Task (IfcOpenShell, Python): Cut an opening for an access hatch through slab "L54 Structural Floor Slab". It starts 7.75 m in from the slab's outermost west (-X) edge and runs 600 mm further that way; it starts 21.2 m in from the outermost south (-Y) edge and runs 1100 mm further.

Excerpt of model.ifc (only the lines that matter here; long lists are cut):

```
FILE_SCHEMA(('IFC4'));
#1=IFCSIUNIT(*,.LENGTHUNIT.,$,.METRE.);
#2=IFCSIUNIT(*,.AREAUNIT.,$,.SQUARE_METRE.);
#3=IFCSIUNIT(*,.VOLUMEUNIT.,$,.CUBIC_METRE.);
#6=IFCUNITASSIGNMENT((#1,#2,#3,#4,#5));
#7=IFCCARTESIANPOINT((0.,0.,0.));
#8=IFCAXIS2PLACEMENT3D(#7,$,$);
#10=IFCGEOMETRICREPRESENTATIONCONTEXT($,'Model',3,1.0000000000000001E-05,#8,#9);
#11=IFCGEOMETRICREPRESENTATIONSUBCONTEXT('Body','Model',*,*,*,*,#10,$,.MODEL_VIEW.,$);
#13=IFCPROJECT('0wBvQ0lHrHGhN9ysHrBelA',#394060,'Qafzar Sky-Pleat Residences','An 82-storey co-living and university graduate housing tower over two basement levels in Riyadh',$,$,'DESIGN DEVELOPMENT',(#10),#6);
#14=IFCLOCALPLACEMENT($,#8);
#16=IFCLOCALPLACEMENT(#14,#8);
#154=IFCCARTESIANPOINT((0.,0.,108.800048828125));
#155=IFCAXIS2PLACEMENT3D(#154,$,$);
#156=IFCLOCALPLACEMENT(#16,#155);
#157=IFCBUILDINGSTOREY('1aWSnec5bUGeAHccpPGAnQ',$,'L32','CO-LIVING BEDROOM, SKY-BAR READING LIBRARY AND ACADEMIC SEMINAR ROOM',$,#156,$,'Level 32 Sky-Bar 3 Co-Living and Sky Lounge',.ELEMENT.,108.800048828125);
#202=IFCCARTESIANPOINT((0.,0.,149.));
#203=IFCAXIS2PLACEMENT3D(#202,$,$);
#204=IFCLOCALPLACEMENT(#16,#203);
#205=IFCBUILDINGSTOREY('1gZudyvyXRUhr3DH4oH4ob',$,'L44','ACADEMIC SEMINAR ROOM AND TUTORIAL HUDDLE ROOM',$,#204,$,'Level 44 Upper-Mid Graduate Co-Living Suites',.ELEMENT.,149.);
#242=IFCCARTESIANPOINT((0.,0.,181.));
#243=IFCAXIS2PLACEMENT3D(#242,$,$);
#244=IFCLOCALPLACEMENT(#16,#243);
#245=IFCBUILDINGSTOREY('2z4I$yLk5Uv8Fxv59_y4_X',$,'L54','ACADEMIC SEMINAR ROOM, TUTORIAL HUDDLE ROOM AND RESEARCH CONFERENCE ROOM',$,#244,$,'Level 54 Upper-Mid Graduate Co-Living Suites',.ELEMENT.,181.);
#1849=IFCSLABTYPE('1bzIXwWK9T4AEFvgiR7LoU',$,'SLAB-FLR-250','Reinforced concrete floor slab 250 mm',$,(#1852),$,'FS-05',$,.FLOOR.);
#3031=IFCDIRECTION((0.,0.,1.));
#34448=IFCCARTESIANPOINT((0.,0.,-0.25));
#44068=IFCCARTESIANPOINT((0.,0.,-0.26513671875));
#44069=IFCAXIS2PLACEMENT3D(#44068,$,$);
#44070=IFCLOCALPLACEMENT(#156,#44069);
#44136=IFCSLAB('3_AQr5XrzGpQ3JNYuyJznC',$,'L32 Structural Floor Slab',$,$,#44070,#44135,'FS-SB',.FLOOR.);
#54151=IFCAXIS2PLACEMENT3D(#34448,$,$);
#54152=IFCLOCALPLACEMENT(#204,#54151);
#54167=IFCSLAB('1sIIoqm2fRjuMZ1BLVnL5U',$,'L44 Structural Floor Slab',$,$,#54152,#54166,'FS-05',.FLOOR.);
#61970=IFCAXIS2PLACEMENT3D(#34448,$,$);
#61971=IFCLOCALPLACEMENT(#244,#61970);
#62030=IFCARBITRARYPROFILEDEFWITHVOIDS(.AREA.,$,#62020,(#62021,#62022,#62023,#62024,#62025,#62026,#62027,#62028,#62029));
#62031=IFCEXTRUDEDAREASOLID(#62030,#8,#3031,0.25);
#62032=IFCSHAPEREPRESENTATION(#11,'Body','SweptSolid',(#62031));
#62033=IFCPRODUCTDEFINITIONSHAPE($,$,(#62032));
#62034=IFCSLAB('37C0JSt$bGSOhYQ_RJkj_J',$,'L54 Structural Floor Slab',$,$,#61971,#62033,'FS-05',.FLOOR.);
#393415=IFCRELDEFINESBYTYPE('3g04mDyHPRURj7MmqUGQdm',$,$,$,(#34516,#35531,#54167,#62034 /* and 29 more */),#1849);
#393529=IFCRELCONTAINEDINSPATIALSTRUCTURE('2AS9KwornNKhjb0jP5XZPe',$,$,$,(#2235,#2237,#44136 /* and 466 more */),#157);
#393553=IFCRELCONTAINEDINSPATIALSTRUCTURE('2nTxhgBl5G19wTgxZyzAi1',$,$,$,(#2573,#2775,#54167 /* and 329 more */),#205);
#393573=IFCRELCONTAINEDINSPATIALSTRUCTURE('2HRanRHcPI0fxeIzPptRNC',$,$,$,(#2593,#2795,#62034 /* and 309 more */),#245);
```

```python
import numpy as np
import ifcopenshell
import ifcopenshell.api.feature
import ifcopenshell.api.geometry
import ifcopenshell.api.root
import ifcopenshell.geom
import ifcopenshell.util.placement
import ifcopenshell.util.representation
import ifcopenshell.util.shape
import ifcopenshell.util.unit

model = ifcopenshell.open("model.ifc")
unit_scale = ifcopenshell.util.unit.calculate_unit_scale(model)
settings = ifcopenshell.geom.settings()


def volume(element):
    """Net volume in cubic metres, openings subtracted."""
    shape = ifcopenshell.geom.create_shape(settings, element)
    return ifcopenshell.util.shape.get_volume(shape.geometry)


slab = model.by_guid("37C0JSt$bGSOhYQ_RJkj_J")
before = volume(slab)

# Extent in the slab's own axes, in metres. The edges named are its -X and -Y sides.
slab_shape = ifcopenshell.geom.create_shape(settings, slab)
vertices = ifcopenshell.util.shape.get_vertices(slab_shape.geometry)
x_min, y_min, bottom = vertices.min(axis=0)
top = vertices[:, 2].max()

opening = ifcopenshell.api.root.create_entity(model, ifc_class="IfcOpeningElement", name="Access hatch opening", predefined_type="OPENING")
context = ifcopenshell.util.representation.get_context(model, "Model", "Body", "MODEL_VIEW")
width, depth = 0.6, 1.1
outline = [(0.0, 0.0), (width, 0.0), (width, depth), (0.0, depth), (0.0, 0.0)]
# Overshoot both faces by 50 mm so the cut is clean.
shape = ifcopenshell.api.geometry.add_slab_representation(
    model, context=context, depth=top - bottom + 0.1, polyline=outline
)
ifcopenshell.api.geometry.assign_representation(model, product=opening, representation=shape)

matrix = ifcopenshell.util.placement.get_local_placement(slab.ObjectPlacement)
matrix[:, 3] = matrix @ np.append(np.array([x_min + 7.75, y_min + 21.2, bottom - 0.05]) / unit_scale, 1.0)
ifcopenshell.api.geometry.edit_object_placement(model, product=opening, matrix=matrix, is_si=False)
ifcopenshell.api.feature.add_feature(model, feature=opening, element=slab)

after = volume(slab)

print(f"slab volume {before:.3f} -> {after:.3f} m3")

model.write("model_v2.ifc")
```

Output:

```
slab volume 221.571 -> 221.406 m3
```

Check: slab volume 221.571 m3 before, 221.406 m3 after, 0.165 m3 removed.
